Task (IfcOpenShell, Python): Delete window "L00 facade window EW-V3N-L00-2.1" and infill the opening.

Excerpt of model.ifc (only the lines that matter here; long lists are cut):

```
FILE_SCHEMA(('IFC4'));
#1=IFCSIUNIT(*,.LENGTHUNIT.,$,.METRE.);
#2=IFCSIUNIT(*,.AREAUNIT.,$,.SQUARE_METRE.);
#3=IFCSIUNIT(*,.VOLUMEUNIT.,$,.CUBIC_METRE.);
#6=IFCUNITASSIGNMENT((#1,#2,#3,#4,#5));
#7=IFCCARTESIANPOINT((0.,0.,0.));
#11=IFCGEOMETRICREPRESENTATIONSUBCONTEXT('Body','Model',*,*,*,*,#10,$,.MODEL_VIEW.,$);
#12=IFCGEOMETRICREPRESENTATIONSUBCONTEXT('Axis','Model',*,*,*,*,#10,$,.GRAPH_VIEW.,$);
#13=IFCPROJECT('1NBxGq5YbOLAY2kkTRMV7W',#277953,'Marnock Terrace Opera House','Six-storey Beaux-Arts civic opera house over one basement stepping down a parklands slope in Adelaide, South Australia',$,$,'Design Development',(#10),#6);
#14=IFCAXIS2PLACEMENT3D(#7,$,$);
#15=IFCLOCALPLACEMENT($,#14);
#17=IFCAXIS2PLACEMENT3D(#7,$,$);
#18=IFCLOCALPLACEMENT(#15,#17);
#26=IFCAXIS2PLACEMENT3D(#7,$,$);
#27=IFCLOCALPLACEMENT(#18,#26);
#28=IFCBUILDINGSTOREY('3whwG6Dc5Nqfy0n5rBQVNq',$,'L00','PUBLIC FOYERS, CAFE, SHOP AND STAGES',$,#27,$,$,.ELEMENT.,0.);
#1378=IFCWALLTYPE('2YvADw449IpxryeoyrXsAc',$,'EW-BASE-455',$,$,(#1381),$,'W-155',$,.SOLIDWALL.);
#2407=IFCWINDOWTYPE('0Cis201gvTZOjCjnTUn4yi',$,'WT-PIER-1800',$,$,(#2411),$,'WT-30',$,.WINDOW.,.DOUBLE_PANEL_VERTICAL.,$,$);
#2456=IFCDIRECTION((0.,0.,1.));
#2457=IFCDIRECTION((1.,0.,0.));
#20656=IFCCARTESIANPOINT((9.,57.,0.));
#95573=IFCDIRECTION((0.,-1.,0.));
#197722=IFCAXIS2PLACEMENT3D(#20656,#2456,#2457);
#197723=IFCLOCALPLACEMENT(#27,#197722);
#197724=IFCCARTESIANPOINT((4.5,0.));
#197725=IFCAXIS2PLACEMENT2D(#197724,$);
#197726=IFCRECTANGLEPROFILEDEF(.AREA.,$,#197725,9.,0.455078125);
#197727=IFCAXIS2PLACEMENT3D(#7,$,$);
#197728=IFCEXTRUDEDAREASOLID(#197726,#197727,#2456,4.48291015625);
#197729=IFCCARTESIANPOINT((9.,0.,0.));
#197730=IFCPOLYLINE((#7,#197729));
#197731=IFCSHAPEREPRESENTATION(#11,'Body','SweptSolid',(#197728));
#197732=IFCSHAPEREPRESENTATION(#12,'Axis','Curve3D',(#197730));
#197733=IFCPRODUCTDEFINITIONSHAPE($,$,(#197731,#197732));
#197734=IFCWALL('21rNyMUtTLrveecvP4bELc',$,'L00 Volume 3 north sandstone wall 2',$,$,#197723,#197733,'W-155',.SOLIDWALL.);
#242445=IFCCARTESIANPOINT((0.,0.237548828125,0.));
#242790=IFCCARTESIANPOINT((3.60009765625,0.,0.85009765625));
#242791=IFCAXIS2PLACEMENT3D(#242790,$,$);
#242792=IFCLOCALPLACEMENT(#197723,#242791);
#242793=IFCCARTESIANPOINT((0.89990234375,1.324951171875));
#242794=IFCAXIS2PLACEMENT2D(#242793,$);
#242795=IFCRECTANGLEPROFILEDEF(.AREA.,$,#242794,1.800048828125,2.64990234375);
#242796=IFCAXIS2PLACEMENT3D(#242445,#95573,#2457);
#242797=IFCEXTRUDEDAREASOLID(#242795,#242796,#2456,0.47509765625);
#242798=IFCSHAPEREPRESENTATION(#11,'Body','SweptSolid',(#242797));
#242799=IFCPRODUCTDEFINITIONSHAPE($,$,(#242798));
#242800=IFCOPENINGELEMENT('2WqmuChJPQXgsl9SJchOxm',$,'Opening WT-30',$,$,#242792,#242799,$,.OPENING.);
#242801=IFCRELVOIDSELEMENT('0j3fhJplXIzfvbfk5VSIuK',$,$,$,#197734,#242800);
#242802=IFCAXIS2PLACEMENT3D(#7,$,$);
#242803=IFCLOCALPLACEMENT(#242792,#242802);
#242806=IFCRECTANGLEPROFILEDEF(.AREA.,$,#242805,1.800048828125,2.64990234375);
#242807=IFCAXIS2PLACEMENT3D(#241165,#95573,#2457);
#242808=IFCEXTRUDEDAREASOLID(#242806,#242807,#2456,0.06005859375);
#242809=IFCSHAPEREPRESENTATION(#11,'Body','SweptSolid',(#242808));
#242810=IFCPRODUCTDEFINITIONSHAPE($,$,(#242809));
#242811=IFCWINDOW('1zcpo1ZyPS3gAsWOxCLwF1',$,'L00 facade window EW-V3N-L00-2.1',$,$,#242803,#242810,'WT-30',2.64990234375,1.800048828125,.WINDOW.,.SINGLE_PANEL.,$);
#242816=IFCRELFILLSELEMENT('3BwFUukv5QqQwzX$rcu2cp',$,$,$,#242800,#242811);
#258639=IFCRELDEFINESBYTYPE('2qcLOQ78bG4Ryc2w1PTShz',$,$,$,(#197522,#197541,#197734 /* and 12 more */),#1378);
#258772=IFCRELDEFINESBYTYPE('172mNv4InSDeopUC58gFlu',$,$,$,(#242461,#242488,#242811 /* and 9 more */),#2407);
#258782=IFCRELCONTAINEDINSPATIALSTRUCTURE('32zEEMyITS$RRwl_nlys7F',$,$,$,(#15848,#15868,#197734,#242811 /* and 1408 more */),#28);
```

```python
import ifcopenshell
import ifcopenshell.api.feature
import ifcopenshell.api.root
import ifcopenshell.geom
import ifcopenshell.util.shape

model = ifcopenshell.open("model.ifc")
settings = ifcopenshell.geom.settings()


def volume(element):
    """Net volume in cubic metres, openings subtracted."""
    shape = ifcopenshell.geom.create_shape(settings, element)
    return ifcopenshell.util.shape.get_volume(shape.geometry)


window = model.by_guid("1zcpo1ZyPS3gAsWOxCLwF1")
opening = window.FillsVoids[0].RelatingOpeningElement
wall = opening.VoidsElements[0].RelatingBuildingElement
before = volume(wall)

ifcopenshell.api.root.remove_product(model, product=window)
ifcopenshell.api.feature.remove_feature(model, feature=opening)

after = volume(wall)

print(f"wall volume {before:.3f} -> {after:.3f} m3")

model.write("model_updated.ifc")
```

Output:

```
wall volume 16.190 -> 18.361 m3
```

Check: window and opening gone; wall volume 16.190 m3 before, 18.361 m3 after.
